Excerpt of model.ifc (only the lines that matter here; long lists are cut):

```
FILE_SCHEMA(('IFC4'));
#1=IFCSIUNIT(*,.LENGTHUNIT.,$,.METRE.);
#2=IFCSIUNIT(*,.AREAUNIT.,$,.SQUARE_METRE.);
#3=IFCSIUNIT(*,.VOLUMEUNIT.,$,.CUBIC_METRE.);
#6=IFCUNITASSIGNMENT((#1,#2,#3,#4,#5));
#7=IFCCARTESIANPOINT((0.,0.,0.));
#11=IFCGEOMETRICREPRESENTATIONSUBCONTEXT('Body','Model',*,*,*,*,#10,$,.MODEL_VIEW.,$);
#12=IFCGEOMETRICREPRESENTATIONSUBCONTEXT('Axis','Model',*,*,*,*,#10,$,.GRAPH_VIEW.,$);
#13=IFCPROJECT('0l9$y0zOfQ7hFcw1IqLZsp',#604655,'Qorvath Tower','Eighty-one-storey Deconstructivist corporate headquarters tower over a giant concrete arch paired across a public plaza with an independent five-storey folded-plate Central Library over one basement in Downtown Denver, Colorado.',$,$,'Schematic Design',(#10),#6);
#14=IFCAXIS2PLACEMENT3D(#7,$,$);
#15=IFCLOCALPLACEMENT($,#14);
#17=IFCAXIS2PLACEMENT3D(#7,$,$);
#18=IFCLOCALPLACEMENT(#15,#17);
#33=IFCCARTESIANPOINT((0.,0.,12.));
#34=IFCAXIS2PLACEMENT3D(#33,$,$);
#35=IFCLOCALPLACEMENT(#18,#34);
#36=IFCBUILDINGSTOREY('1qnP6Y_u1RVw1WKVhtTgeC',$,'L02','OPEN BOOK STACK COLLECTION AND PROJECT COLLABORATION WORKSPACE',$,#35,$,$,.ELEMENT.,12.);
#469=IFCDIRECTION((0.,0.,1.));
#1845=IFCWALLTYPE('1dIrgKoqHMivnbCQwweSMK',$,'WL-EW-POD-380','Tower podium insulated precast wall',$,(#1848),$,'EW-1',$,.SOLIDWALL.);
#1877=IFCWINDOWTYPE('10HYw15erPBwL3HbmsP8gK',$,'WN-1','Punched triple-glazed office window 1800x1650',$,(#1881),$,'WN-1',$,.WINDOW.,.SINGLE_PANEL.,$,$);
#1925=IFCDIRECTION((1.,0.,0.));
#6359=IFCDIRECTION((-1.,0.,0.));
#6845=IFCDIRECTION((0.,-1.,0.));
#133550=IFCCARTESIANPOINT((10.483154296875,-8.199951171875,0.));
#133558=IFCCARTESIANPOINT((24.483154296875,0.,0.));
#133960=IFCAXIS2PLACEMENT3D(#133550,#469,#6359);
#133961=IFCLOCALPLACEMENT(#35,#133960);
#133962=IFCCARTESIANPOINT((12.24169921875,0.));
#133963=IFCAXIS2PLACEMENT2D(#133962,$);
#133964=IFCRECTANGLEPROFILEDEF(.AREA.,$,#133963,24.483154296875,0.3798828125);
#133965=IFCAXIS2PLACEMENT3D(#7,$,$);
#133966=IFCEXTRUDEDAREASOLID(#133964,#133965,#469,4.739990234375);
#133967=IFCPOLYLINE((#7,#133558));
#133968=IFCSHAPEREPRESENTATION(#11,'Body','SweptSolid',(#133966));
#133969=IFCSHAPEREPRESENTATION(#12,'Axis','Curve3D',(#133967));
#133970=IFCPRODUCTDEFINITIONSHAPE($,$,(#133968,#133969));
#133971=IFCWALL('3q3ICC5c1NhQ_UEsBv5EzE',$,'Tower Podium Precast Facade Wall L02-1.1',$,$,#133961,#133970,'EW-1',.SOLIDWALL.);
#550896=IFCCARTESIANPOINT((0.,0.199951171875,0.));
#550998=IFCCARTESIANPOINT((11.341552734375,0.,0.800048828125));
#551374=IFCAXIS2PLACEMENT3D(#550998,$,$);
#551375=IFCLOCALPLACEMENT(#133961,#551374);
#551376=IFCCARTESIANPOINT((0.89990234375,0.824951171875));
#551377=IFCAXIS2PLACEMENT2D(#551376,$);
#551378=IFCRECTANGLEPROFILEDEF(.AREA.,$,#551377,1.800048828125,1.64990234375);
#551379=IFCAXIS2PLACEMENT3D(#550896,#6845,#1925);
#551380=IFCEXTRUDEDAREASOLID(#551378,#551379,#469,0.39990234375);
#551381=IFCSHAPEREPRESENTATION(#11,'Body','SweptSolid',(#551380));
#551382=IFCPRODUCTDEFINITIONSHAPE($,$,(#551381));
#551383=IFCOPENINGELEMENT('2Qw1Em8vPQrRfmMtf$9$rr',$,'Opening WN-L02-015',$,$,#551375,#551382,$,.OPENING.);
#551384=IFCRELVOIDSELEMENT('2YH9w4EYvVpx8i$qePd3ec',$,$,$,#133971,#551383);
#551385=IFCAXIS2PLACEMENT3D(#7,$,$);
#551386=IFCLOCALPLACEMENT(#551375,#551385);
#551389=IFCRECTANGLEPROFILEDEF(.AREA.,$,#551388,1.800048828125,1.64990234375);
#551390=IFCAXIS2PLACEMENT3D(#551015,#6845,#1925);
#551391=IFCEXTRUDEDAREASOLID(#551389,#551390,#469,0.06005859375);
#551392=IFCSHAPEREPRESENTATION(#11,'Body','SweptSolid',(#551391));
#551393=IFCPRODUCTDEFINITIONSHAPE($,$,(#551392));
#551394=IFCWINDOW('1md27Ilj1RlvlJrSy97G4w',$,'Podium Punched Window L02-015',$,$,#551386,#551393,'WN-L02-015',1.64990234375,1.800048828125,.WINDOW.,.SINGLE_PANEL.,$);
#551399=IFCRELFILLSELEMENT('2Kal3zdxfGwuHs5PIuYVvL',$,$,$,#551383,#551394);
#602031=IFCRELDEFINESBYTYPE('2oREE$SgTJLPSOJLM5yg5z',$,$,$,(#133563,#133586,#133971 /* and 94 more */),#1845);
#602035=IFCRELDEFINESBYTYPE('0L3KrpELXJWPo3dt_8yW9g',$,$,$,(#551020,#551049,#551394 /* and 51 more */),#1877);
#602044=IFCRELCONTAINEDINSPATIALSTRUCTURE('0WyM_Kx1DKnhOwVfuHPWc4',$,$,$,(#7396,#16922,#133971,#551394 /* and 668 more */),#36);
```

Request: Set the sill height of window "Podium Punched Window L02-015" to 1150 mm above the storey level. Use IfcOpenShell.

```python
import numpy as np
import ifcopenshell
import ifcopenshell.api.geometry
import ifcopenshell.geom
import ifcopenshell.util.element
import ifcopenshell.util.placement
import ifcopenshell.util.shape
import ifcopenshell.util.unit

model = ifcopenshell.open("model.ifc")
unit_scale = ifcopenshell.util.unit.calculate_unit_scale(model)

window = model.by_guid("1md27Ilj1RlvlJrSy97G4w")
opening = window.FillsVoids[0].RelatingOpeningElement
storey = ifcopenshell.util.element.get_container(window, ifc_class="IfcBuildingStorey")
level = ifcopenshell.util.placement.get_local_placement(storey.ObjectPlacement)[2, 3]

# The opening's origin need not be at the sill, so measure its lowest point.
shape = ifcopenshell.geom.create_shape(ifcopenshell.geom.settings(), opening)
bottom = ifcopenshell.util.shape.get_shape_bottom_elevation(shape, shape.geometry) / unit_scale
dz = level + 1.15 - bottom

shift = np.array([0.0, 0.0, dz])
# The window is placed relative to its opening, so it follows when the opening moves.
matrix = ifcopenshell.util.placement.get_local_placement(opening.ObjectPlacement)
matrix[:3, 3] += shift
ifcopenshell.api.geometry.edit_object_placement(
    model, product=opening, matrix=matrix, is_si=False, should_transform_children=True
)

print(f"moved by {dz * unit_scale:+.3f} m")

model.write("model_rev.ifc")
```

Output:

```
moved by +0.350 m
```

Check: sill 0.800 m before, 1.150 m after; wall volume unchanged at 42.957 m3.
